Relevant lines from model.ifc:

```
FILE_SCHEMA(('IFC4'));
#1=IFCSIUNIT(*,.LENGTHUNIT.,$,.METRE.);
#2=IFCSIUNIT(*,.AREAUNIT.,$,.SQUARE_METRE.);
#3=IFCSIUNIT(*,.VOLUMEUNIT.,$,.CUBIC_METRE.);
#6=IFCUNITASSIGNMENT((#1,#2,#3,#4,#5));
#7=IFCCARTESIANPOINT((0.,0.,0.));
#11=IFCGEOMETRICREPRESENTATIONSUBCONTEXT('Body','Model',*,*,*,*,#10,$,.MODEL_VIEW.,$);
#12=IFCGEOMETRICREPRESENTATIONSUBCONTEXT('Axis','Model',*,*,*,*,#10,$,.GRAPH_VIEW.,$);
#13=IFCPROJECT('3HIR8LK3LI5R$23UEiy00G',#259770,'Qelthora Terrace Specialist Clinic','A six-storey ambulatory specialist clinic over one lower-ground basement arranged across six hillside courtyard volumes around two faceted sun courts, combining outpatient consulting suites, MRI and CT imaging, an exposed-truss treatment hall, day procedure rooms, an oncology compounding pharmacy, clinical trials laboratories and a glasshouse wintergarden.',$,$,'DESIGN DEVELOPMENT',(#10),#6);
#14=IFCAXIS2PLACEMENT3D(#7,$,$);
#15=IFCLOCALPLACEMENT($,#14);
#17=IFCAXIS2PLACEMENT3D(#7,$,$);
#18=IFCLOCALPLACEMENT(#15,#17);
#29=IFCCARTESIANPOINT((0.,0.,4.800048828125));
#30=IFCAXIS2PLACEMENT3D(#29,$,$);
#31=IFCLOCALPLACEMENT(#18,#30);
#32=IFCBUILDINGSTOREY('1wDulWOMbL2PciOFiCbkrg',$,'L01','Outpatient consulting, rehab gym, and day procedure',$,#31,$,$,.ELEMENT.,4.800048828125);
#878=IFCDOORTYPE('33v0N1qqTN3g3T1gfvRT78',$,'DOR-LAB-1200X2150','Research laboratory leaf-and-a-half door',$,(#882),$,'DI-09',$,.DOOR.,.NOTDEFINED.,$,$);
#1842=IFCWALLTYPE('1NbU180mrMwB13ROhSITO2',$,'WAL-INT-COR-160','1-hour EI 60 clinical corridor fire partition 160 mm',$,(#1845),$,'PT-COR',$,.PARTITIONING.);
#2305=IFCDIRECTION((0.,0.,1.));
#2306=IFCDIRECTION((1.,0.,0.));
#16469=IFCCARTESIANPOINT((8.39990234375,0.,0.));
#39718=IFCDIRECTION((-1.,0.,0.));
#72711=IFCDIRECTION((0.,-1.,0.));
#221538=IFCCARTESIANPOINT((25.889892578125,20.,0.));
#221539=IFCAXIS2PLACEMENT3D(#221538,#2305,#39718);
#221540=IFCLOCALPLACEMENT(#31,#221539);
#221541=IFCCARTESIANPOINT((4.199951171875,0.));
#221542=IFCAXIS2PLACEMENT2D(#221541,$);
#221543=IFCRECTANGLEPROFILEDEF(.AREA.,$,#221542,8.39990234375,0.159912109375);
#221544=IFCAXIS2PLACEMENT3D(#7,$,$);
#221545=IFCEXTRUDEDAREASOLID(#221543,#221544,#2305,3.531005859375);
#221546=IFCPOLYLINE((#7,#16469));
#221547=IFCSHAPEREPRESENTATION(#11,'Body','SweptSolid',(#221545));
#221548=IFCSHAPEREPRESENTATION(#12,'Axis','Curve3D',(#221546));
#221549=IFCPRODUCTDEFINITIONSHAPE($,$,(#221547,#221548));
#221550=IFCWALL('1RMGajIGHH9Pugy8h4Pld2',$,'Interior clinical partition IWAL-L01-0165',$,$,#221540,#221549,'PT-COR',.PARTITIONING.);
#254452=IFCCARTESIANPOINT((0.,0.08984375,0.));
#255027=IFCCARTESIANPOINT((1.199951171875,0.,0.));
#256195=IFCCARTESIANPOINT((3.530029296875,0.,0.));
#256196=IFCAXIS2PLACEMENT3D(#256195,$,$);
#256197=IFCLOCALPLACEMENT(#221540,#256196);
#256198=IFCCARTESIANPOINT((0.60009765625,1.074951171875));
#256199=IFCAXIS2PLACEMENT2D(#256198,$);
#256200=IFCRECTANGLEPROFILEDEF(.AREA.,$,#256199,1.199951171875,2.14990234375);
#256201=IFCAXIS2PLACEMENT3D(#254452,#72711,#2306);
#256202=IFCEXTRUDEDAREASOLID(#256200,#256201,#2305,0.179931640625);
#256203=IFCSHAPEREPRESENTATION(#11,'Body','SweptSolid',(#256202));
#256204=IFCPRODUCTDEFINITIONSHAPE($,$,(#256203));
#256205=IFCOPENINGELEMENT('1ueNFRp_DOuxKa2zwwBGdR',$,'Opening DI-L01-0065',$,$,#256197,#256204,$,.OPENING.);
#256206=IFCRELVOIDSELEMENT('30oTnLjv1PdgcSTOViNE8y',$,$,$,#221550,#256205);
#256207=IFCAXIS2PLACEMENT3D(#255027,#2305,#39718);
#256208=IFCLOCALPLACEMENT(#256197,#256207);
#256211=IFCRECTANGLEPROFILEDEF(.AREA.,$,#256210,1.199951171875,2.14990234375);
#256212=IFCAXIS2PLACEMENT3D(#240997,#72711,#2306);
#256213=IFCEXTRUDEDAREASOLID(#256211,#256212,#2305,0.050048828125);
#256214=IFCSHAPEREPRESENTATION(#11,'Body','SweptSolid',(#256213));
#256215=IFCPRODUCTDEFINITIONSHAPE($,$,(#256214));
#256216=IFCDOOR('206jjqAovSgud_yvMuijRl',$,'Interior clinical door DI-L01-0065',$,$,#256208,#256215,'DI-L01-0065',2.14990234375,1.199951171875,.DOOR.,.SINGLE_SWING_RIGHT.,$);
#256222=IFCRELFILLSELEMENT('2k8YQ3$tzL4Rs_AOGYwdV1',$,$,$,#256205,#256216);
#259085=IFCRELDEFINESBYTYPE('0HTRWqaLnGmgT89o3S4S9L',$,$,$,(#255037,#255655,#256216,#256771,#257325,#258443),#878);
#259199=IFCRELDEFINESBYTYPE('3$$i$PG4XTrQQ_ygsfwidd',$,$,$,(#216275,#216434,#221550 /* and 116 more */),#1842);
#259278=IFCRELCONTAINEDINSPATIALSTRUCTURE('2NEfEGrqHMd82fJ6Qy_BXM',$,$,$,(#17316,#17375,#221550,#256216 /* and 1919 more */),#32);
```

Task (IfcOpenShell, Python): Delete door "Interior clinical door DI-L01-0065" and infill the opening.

```python
import ifcopenshell
import ifcopenshell.api.feature
import ifcopenshell.api.root
import ifcopenshell.geom
import ifcopenshell.util.shape

model = ifcopenshell.open("model.ifc")
settings = ifcopenshell.geom.settings()


def volume(element):
    """Net volume in cubic metres, openings subtracted."""
    shape = ifcopenshell.geom.create_shape(settings, element)
    return ifcopenshell.util.shape.get_volume(shape.geometry)


door = model.by_guid("206jjqAovSgud_yvMuijRl")
opening = door.FillsVoids[0].RelatingOpeningElement
wall = opening.VoidsElements[0].RelatingBuildingElement
before = volume(wall)

ifcopenshell.api.root.remove_product(model, product=door)
ifcopenshell.api.feature.remove_feature(model, feature=opening)

after = volume(wall)

print(f"wall volume {before:.3f} -> {after:.3f} m3")

model.write("model-out.ifc")
```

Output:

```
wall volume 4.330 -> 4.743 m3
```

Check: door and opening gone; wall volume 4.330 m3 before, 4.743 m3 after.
